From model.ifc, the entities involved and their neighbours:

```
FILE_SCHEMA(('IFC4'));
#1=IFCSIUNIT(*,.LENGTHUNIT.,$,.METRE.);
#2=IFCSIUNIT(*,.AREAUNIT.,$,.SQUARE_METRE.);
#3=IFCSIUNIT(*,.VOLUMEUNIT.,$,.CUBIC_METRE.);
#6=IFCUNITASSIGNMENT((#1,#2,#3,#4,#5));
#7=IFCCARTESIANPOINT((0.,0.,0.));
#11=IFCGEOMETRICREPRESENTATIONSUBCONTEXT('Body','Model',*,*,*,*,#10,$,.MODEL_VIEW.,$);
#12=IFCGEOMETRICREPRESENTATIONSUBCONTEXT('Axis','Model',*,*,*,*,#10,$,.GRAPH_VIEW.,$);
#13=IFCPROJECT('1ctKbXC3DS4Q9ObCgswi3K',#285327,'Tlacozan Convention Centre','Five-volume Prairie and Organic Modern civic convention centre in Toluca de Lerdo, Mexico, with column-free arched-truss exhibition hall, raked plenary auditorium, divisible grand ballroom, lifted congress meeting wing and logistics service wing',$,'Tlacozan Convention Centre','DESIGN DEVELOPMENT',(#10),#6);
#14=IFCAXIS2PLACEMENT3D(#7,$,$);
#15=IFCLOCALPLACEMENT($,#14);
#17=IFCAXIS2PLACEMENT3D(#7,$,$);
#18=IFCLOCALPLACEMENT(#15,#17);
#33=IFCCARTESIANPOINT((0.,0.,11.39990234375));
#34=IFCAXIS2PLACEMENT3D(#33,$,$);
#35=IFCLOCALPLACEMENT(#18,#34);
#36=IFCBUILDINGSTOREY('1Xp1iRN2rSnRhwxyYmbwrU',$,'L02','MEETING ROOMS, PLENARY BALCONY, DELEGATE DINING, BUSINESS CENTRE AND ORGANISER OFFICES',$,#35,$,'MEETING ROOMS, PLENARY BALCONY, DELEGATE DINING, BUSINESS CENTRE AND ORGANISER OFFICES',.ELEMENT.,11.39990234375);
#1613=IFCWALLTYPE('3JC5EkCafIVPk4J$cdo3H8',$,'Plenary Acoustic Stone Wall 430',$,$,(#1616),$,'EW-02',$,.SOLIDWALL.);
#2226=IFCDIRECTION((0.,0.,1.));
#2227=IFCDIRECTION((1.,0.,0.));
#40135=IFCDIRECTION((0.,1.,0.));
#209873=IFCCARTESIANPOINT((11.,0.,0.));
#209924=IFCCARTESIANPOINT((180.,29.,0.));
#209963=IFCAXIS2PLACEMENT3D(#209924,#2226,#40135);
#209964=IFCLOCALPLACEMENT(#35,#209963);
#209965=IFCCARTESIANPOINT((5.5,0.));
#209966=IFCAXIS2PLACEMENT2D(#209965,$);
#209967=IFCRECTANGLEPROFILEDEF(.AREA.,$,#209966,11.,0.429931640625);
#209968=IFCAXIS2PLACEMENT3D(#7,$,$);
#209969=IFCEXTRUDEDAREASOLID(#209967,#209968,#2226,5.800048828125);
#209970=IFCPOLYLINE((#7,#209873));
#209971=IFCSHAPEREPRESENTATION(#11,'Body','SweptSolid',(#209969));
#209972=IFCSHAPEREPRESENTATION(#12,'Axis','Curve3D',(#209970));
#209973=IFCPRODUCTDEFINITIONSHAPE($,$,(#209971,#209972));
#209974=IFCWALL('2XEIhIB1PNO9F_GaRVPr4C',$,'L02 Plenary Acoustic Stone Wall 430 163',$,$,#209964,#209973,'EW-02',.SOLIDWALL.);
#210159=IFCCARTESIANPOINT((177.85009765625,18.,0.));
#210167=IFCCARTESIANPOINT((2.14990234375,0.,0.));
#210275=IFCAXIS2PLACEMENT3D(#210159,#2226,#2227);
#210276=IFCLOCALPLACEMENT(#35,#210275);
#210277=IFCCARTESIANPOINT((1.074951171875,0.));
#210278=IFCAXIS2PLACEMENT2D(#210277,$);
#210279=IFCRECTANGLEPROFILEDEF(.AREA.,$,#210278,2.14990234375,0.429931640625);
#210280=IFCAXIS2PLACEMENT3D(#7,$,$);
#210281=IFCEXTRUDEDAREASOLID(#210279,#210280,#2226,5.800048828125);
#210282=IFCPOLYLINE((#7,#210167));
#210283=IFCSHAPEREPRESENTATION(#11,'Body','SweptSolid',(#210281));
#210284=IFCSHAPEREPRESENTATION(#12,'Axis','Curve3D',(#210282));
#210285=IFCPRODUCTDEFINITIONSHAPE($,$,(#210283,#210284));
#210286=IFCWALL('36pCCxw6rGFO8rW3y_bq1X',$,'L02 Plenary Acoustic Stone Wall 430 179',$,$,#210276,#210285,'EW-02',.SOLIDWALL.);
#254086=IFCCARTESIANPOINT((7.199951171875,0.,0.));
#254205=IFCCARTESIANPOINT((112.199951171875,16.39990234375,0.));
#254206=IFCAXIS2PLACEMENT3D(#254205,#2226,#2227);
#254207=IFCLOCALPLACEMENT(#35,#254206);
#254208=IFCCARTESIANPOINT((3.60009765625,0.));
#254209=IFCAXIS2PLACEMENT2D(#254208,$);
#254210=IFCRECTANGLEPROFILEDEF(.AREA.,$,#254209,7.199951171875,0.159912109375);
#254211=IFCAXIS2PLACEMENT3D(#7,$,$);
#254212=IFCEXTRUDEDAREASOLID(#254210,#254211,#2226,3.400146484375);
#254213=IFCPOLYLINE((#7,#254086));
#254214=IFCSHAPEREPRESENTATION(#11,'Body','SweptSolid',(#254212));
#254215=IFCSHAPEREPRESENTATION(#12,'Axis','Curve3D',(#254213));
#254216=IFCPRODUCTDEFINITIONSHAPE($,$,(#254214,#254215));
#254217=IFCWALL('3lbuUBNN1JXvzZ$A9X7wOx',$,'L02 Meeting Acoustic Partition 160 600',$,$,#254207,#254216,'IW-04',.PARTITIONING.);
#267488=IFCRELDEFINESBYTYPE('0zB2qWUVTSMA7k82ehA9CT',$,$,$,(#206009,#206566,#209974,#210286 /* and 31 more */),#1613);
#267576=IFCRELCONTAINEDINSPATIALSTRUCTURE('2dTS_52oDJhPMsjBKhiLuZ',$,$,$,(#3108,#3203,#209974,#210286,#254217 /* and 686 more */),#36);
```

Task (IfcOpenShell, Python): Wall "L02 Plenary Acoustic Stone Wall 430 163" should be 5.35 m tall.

```python
import ifcopenshell
import ifcopenshell.geom
import ifcopenshell.util.representation
import ifcopenshell.util.shape

model = ifcopenshell.open("model.ifc")
settings = ifcopenshell.geom.settings()


def volume(element):
    """Net volume in cubic metres, openings subtracted."""
    shape = ifcopenshell.geom.create_shape(settings, element)
    return ifcopenshell.util.shape.get_volume(shape.geometry)


wall = model.by_guid("2XEIhIB1PNO9F_GaRVPr4C")
before = volume(wall)

body = ifcopenshell.util.representation.get_representation(wall, "Model", "Body")
solid = body.Items[0]
old_height = solid.Depth
solid.Depth = 5.35
after = volume(wall)

print(f"height {old_height:g} -> {solid.Depth:g}, volume {before:.3f} -> {after:.3f} m3")

model.write("model-out.ifc")
```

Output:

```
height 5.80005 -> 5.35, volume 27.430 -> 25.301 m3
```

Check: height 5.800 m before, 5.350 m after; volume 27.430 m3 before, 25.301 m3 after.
